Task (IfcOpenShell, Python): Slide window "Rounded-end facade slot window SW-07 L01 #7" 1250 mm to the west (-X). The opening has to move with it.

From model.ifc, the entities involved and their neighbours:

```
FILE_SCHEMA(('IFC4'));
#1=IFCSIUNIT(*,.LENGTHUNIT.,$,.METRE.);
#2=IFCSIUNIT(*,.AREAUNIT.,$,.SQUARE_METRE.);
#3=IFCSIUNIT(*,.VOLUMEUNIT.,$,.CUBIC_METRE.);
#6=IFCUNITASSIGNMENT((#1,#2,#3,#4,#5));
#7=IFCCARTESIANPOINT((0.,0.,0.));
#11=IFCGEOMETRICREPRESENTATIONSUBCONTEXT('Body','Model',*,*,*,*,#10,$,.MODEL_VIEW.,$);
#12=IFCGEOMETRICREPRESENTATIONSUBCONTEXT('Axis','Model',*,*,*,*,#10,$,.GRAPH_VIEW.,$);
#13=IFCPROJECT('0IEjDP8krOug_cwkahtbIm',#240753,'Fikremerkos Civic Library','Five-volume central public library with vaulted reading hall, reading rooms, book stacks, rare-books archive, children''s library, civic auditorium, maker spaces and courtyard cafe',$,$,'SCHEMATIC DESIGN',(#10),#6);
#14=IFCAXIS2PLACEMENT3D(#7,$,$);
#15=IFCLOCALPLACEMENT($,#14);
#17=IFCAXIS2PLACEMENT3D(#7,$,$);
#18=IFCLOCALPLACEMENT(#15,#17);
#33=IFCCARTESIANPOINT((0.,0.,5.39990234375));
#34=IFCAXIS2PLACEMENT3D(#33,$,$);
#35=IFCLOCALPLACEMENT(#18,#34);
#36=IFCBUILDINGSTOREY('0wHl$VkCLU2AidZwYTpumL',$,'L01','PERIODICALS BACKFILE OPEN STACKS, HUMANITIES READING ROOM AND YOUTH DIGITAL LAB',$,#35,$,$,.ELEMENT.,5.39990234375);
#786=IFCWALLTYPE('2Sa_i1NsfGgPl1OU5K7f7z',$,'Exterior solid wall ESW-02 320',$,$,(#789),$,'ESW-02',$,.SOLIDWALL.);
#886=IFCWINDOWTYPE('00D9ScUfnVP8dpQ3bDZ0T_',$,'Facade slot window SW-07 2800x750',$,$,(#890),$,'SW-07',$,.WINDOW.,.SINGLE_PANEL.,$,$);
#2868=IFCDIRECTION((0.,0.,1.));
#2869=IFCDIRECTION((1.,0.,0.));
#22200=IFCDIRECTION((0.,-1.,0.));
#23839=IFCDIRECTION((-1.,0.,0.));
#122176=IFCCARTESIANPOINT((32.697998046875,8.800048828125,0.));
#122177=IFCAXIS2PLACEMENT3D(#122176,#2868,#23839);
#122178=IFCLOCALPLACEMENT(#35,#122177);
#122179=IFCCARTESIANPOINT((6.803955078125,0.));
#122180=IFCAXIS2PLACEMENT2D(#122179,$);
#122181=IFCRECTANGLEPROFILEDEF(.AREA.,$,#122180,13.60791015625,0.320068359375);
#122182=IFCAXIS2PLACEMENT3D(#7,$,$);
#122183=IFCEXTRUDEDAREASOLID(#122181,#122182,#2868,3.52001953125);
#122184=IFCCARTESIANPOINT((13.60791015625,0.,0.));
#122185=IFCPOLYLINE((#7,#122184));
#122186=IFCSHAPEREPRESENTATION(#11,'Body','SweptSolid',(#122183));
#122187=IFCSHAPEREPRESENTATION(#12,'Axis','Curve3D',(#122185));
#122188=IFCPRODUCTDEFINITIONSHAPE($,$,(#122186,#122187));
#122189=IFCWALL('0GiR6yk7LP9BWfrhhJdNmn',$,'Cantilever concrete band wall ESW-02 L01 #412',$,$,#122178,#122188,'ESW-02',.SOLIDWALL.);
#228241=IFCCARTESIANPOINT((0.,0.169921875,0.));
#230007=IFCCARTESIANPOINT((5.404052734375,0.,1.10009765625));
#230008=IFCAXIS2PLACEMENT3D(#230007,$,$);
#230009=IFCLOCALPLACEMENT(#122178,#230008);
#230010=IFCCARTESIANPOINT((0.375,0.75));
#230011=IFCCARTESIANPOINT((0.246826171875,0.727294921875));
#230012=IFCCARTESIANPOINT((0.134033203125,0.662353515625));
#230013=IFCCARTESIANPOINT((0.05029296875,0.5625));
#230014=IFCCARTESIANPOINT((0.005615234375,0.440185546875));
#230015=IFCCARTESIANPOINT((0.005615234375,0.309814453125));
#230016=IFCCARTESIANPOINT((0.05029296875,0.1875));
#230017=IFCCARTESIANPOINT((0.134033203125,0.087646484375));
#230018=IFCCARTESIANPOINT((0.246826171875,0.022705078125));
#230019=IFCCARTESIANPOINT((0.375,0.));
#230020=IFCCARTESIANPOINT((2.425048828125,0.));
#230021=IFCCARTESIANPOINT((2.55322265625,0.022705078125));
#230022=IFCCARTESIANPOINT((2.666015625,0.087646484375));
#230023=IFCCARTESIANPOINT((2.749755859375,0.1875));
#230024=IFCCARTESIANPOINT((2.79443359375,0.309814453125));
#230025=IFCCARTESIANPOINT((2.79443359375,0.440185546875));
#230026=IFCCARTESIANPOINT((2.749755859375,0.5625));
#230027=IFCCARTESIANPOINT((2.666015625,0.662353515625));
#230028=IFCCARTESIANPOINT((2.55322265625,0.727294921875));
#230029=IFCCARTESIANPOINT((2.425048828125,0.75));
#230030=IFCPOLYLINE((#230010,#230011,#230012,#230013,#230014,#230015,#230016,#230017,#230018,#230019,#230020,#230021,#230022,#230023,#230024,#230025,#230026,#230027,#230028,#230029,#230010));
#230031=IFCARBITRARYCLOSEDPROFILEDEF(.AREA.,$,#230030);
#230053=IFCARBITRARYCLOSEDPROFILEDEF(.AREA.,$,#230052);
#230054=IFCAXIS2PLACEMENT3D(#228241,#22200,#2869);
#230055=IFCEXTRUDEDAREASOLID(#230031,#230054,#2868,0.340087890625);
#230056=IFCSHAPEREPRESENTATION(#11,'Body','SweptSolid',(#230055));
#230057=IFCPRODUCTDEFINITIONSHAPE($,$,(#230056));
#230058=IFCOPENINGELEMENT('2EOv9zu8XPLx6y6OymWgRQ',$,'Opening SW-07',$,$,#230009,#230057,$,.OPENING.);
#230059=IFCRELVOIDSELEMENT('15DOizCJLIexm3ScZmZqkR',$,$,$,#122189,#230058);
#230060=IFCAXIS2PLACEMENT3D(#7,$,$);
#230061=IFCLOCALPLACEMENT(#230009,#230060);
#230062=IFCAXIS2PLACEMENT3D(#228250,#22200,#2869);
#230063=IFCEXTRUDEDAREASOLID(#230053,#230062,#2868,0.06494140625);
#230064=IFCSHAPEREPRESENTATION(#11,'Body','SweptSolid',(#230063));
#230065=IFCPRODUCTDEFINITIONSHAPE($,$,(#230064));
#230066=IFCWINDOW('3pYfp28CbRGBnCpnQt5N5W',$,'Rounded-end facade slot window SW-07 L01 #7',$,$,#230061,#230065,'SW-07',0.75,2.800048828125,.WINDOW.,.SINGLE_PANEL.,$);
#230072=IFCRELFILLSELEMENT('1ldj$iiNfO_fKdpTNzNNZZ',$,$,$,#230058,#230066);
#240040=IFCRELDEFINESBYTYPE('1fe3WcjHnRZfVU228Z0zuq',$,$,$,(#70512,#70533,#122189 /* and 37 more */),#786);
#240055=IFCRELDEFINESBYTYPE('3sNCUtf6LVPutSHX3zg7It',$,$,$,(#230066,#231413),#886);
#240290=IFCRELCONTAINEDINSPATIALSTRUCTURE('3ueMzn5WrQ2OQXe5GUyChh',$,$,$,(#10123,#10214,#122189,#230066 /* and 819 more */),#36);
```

```python
import ifcopenshell
import ifcopenshell.api.geometry
import ifcopenshell.util.placement

model = ifcopenshell.open("model.ifc")

window = model.by_id(230066)
opening = window.FillsVoids[0].RelatingOpeningElement
wall = opening.VoidsElements[0].RelatingBuildingElement

wall_matrix = ifcopenshell.util.placement.get_local_placement(wall.ObjectPlacement)
shift = wall_matrix[:3, 0] * 1.25
before = ifcopenshell.util.placement.get_local_placement(window.ObjectPlacement)[:3, 3].copy()

# The window is placed relative to its opening, so it follows when the opening moves.
matrix = ifcopenshell.util.placement.get_local_placement(opening.ObjectPlacement)
matrix[:3, 3] += shift
ifcopenshell.api.geometry.edit_object_placement(
    model, product=opening, matrix=matrix, is_si=False, should_transform_children=True
)

after = ifcopenshell.util.placement.get_local_placement(window.ObjectPlacement)[:3, 3]
print("window moved by", (after - before).round(3) + 0.0)

model.write("model-out.ifc")
```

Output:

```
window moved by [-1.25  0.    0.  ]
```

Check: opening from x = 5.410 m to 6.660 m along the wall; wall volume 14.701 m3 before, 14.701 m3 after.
